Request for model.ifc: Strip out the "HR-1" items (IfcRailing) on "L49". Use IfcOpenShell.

First a look at what the model holds.

```python
import ifcopenshell
import ifcopenshell.util.element

model = ifcopenshell.open("model.ifc")
print(model.schema)
storey = next(s for s in model.by_type("IfcBuildingStorey") if s.Name == "L49")
railings = [e for e in ifcopenshell.util.element.get_decomposition(storey) if e.is_a("IfcRailing")]
seen = {}
for e in railings:
    element_type = ifcopenshell.util.element.get_type(e)
    name = element_type.Name if element_type not in (None, e) else None
    seen[name] = seen.get(name, 0) + 1
for name, count in sorted(seen.items(), key=str):
    print(count, "x", name)
```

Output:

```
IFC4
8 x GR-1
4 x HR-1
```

```python
import ifcopenshell
import ifcopenshell.api.root
import ifcopenshell.util.element

model = ifcopenshell.open("model.ifc")

storey = next(s for s in model.by_type("IfcBuildingStorey") if s.Name == "L49")
railings = [e for e in ifcopenshell.util.element.get_decomposition(storey) if e.is_a("IfcRailing")]
targets = [e for e in railings if (t := ifcopenshell.util.element.get_type(e)) not in (None, e) and t.Name == "HR-1"]

for e in targets:
    ifcopenshell.api.root.remove_product(model, product=e)
print(len(targets), "removed")

model.write("model-out.ifc")
```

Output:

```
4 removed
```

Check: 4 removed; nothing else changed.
